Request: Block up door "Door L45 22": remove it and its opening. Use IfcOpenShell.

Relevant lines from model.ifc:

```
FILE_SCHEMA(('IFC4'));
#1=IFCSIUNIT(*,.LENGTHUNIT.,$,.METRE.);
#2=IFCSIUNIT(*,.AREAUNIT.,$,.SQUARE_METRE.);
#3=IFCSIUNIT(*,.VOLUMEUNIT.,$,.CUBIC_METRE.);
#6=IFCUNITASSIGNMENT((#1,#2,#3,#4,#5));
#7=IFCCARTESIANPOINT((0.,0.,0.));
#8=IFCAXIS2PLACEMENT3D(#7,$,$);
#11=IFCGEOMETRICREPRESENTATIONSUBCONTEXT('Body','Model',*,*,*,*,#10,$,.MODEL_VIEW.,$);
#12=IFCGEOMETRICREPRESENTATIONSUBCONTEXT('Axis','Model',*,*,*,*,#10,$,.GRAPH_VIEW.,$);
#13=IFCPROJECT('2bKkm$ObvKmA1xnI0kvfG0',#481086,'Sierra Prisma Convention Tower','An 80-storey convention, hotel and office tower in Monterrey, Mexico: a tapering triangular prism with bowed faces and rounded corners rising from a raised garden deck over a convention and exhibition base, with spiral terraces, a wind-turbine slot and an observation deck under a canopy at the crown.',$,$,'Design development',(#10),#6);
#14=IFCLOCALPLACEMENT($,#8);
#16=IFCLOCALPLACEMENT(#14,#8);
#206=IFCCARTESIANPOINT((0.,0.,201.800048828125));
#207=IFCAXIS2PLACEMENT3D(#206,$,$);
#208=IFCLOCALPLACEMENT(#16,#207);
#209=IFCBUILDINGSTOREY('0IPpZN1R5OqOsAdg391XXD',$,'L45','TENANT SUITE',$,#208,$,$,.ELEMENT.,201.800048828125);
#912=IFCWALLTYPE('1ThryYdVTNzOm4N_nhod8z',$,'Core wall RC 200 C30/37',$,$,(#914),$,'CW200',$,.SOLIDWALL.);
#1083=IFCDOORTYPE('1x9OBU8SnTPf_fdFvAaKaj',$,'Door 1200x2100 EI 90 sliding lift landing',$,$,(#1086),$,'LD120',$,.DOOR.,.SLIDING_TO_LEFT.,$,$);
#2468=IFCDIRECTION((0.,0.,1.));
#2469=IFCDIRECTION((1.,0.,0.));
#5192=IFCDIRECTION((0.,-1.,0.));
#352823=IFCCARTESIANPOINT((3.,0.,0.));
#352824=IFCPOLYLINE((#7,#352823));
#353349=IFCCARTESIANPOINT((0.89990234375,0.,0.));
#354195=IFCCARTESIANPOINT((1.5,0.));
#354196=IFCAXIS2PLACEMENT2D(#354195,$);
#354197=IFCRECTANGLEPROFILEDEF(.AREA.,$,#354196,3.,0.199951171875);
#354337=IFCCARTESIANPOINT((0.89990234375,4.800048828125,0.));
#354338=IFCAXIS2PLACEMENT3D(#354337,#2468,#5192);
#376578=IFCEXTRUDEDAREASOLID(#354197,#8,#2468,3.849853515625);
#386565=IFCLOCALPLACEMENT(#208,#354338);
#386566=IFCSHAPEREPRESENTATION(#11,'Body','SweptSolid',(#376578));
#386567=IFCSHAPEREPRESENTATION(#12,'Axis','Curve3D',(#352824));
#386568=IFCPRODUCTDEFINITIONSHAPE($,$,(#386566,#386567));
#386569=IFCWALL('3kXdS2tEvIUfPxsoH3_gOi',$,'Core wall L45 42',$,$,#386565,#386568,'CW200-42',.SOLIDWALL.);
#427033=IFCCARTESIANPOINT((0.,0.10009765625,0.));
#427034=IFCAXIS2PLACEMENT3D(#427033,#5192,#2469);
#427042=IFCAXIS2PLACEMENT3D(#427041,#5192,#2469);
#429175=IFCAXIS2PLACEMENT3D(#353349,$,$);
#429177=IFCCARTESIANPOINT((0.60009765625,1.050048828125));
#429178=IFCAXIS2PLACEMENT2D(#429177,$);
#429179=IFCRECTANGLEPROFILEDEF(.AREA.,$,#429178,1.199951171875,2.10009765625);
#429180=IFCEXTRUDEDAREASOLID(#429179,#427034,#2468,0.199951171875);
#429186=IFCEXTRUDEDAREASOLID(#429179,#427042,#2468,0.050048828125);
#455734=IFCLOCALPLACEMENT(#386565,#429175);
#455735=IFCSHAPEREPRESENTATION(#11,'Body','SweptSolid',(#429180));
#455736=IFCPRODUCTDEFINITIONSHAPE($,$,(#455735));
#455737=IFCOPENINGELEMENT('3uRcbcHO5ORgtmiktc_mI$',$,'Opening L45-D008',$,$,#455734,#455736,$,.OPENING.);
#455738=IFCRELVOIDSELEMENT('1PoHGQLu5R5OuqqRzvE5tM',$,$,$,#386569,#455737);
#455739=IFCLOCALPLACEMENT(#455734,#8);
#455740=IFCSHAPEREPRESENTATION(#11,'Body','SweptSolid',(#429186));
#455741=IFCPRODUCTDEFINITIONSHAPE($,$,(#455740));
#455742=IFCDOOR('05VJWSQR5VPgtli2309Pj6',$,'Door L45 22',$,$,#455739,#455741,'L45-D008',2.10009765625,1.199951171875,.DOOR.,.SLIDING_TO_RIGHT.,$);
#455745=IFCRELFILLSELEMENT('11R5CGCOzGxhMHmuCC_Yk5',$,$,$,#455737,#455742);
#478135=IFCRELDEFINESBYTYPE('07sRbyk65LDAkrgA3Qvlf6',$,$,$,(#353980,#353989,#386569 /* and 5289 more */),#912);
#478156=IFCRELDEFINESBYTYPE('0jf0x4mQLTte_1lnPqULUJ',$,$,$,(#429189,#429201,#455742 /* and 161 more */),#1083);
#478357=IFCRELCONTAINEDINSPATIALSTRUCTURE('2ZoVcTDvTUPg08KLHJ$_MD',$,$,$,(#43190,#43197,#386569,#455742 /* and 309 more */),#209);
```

```python
import ifcopenshell
import ifcopenshell.api.feature
import ifcopenshell.api.root
import ifcopenshell.geom
import ifcopenshell.util.shape

model = ifcopenshell.open("model.ifc")
settings = ifcopenshell.geom.settings()


def volume(element):
    """Net volume in cubic metres, openings subtracted."""
    shape = ifcopenshell.geom.create_shape(settings, element)
    return ifcopenshell.util.shape.get_volume(shape.geometry)


door = model.by_guid("05VJWSQR5VPgtli2309Pj6")
opening = door.FillsVoids[0].RelatingOpeningElement
wall = opening.VoidsElements[0].RelatingBuildingElement
before = volume(wall)

ifcopenshell.api.root.remove_product(model, product=door)
ifcopenshell.api.feature.remove_feature(model, feature=opening)

after = volume(wall)

print(f"wall volume {before:.3f} -> {after:.3f} m3")

model.write("model_v2.ifc")
```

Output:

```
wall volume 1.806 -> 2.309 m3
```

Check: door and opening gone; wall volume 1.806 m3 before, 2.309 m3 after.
